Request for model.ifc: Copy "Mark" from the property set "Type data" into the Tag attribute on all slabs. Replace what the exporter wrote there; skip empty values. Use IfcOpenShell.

First a look at what the model holds.

```python
import ifcopenshell
import ifcopenshell.util.element

model = ifcopenshell.open("model.ifc")
print(model.schema)
slabs = model.by_type("IfcSlab")
print(len(slabs), "slabs")
for e in slabs[:8]:
    source = ifcopenshell.util.element.get_pset(e, "Type data", "Mark")
    target = e.Tag
    print(e.id(), repr(source), repr(target), sep=" | ")
```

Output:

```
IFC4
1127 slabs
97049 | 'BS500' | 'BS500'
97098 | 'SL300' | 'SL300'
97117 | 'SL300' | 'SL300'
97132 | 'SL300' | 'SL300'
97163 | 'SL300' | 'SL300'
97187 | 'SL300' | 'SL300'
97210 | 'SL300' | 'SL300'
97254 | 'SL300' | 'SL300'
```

```python
import ifcopenshell
import ifcopenshell.util.element

model = ifcopenshell.open("model.ifc")

count = 0
for e in model.by_type("IfcSlab"):
    value = ifcopenshell.util.element.get_pset(e, "Type data", "Mark")
    current = e.Tag
    if not value or not value.strip() or current == value:
        continue
    e.Tag = value
    count += 1

print(count, "slabs updated")

model.write("model_rev.ifc")
```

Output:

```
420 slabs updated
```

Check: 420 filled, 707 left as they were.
